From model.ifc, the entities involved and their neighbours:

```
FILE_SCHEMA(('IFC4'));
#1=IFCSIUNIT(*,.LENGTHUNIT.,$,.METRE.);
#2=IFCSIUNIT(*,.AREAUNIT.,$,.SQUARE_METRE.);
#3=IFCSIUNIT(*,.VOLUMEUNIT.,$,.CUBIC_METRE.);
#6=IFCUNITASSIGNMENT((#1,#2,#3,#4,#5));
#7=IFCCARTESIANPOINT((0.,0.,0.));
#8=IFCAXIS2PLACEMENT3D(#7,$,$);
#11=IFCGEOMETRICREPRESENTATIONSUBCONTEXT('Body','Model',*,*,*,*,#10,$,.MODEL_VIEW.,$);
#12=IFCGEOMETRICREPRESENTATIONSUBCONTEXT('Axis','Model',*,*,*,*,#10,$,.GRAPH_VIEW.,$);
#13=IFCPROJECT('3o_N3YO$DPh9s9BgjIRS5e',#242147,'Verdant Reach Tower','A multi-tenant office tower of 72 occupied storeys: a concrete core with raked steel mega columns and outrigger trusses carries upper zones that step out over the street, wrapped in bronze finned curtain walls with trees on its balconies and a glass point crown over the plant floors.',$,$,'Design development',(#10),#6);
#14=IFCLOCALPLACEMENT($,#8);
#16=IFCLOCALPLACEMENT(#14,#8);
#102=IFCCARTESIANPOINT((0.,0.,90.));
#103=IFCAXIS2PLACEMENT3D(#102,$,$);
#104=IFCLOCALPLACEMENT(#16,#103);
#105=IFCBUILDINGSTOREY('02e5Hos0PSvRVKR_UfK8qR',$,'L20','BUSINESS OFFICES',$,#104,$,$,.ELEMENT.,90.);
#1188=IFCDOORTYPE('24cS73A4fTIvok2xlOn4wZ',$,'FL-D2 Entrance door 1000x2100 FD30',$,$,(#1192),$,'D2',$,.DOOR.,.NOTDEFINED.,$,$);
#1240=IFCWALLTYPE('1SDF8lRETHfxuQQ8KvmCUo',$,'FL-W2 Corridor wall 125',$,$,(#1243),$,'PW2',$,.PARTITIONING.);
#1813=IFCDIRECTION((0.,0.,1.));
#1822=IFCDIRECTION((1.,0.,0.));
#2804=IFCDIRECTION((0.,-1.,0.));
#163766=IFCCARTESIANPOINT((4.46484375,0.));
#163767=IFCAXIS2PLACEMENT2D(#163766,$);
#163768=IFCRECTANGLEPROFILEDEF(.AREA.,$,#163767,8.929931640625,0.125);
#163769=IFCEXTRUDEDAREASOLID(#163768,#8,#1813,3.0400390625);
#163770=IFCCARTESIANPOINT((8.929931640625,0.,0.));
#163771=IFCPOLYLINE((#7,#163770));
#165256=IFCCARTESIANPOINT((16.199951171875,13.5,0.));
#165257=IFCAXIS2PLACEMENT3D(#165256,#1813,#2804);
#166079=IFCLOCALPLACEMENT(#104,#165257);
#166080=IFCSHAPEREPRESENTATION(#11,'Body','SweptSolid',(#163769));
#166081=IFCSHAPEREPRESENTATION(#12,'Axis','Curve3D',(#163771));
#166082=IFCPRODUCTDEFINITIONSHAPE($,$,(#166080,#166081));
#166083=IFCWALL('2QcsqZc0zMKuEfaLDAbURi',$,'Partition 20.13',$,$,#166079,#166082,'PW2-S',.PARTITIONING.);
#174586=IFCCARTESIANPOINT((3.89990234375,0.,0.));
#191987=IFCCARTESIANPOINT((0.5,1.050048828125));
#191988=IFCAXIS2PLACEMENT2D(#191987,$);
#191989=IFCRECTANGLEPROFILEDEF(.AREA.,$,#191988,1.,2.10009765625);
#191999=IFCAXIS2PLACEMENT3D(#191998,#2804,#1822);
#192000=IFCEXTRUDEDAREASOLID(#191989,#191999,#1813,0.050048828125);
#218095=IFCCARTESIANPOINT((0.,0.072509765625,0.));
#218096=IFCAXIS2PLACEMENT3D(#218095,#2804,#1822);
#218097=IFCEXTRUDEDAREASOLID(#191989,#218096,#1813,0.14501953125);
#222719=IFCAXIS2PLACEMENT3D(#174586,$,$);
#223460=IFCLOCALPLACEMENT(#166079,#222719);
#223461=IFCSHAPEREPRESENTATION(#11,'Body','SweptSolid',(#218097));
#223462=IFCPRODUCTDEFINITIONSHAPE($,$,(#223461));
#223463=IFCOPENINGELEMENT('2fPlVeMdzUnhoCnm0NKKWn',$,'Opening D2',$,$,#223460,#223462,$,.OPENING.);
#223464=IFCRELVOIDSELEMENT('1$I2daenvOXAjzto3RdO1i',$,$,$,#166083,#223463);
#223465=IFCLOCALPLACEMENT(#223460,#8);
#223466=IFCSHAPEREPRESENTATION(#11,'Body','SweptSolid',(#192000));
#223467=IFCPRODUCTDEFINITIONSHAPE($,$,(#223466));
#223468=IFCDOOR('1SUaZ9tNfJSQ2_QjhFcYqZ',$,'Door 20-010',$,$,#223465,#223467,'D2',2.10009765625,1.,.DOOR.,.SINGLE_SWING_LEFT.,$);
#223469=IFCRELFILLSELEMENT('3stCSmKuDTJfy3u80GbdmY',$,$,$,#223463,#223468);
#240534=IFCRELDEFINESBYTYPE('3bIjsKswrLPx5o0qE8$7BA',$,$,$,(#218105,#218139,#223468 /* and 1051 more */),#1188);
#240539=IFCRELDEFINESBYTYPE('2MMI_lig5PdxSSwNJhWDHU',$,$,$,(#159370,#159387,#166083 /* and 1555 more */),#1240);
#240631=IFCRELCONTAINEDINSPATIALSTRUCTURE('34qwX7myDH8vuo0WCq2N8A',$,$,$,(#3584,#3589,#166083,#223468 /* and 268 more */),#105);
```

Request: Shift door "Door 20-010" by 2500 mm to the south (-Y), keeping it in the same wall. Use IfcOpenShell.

```python
import ifcopenshell
import ifcopenshell.api.geometry
import ifcopenshell.util.placement

model = ifcopenshell.open("model.ifc")

door = model.by_guid("1SUaZ9tNfJSQ2_QjhFcYqZ")
opening = door.FillsVoids[0].RelatingOpeningElement
wall = opening.VoidsElements[0].RelatingBuildingElement

wall_matrix = ifcopenshell.util.placement.get_local_placement(wall.ObjectPlacement)
shift = wall_matrix[:3, 0] * 2.5
before = ifcopenshell.util.placement.get_local_placement(door.ObjectPlacement)[:3, 3].copy()

# The door is placed relative to its opening, so it follows when the opening moves.
matrix = ifcopenshell.util.placement.get_local_placement(opening.ObjectPlacement)
matrix[:3, 3] += shift
ifcopenshell.api.geometry.edit_object_placement(
    model, product=opening, matrix=matrix, is_si=False, should_transform_children=True
)

after = ifcopenshell.util.placement.get_local_placement(door.ObjectPlacement)[:3, 3]
print("door moved by", (after - before).round(3) + 0.0)

model.write("model_updated.ifc")
```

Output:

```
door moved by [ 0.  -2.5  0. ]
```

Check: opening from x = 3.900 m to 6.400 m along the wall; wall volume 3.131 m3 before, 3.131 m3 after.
